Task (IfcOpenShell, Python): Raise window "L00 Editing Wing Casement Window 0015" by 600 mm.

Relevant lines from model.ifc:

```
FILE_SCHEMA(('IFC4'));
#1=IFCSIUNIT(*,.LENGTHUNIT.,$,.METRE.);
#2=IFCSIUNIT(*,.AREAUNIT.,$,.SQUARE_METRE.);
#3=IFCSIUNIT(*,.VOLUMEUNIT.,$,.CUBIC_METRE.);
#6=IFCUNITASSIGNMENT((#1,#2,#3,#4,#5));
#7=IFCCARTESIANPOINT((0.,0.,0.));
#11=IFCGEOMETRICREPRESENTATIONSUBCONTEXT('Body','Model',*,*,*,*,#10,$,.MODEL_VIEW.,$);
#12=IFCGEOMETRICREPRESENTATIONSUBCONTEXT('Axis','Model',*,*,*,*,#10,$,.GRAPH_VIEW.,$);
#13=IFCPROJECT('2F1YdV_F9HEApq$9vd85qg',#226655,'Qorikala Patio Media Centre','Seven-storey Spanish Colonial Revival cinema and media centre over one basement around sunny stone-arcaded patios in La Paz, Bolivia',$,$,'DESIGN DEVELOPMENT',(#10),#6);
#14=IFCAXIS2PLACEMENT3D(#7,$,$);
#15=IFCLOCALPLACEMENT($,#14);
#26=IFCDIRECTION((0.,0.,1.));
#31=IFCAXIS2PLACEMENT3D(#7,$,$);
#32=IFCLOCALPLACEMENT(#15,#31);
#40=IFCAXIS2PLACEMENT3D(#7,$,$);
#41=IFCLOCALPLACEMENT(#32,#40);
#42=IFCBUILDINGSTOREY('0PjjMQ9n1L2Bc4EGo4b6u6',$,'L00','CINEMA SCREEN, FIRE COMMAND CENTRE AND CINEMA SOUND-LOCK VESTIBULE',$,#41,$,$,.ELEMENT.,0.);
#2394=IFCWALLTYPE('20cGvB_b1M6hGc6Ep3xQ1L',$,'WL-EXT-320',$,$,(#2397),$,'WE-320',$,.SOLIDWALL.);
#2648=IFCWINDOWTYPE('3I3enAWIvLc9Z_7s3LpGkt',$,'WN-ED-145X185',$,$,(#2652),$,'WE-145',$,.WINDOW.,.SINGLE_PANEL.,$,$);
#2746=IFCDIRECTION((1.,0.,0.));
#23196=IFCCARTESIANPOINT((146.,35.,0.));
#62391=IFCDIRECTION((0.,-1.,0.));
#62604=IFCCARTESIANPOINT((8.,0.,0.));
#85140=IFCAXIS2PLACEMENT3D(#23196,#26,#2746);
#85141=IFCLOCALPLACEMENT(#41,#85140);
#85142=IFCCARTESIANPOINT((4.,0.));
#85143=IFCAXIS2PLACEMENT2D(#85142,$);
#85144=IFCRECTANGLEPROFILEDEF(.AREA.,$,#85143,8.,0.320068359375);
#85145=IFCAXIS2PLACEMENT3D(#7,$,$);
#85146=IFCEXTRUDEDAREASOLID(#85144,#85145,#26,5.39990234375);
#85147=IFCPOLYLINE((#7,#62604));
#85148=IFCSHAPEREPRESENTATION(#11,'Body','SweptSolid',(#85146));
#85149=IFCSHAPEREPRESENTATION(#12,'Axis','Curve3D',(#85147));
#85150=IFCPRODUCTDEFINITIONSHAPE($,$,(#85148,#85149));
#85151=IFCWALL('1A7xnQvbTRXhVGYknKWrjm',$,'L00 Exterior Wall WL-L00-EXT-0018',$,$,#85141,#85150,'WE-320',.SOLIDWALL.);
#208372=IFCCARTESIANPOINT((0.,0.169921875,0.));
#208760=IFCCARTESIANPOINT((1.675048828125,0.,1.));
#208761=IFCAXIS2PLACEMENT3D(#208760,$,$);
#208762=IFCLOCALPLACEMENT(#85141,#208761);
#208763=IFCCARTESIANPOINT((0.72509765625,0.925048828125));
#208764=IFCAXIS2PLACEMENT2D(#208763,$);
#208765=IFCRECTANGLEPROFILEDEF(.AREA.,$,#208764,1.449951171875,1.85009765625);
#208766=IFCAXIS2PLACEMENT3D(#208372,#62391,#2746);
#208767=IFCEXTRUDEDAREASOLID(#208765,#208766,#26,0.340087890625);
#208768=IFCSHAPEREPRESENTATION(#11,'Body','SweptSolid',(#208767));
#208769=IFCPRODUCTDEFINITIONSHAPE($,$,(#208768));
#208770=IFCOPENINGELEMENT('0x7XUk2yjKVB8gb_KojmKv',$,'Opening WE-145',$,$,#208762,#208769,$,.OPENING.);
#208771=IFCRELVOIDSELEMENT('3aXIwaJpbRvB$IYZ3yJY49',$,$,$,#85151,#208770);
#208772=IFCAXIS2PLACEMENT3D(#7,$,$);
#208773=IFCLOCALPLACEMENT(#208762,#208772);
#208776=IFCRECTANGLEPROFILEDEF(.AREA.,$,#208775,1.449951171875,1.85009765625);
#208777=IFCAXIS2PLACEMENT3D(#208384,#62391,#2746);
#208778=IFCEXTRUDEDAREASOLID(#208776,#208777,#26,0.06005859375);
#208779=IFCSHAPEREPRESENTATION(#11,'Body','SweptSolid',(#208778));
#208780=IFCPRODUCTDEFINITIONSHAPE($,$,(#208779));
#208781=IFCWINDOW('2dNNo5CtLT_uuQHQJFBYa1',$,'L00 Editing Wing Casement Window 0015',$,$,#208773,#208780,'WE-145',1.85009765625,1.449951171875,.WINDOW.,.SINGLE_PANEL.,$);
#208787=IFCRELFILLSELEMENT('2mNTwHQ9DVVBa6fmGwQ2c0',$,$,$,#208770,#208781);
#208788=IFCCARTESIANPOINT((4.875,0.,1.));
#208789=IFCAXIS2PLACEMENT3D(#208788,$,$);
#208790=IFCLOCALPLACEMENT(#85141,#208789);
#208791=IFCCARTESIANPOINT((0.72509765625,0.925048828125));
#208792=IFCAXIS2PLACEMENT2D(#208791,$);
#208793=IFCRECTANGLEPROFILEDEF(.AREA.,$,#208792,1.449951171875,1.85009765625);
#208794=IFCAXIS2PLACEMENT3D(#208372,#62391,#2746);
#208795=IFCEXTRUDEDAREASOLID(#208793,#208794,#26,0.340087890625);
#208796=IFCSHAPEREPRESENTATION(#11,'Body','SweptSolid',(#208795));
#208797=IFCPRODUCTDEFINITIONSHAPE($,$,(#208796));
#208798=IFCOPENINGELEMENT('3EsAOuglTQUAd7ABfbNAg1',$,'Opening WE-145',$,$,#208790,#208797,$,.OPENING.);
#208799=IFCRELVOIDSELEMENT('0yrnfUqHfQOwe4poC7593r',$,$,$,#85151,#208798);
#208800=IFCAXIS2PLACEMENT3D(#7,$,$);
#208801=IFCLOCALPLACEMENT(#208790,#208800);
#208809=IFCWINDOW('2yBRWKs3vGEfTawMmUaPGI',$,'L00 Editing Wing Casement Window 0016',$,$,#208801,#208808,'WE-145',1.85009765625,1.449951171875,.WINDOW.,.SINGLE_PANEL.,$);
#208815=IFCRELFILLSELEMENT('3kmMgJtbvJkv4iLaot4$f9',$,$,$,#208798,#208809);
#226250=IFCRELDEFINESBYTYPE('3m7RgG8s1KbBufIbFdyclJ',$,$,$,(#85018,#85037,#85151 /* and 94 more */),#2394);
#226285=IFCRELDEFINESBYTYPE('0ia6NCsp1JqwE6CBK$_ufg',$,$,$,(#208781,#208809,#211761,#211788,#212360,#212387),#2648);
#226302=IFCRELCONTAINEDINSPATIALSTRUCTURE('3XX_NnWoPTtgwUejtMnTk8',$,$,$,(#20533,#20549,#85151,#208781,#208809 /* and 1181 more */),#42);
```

```python
import numpy as np
import ifcopenshell
import ifcopenshell.api.geometry
import ifcopenshell.util.placement
import ifcopenshell.util.unit

model = ifcopenshell.open("model.ifc")
unit_scale = ifcopenshell.util.unit.calculate_unit_scale(model)

window = model.by_id(208781)
opening = window.FillsVoids[0].RelatingOpeningElement
dz = 0.6

shift = np.array([0.0, 0.0, dz])
# The window is placed relative to its opening, so it follows when the opening moves.
matrix = ifcopenshell.util.placement.get_local_placement(opening.ObjectPlacement)
matrix[:3, 3] += shift
ifcopenshell.api.geometry.edit_object_placement(
    model, product=opening, matrix=matrix, is_si=False, should_transform_children=True
)

print(f"moved by {dz * unit_scale:+.3f} m")

model.write("model_edited.ifc")
```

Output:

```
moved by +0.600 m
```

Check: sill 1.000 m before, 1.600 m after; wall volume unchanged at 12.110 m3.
